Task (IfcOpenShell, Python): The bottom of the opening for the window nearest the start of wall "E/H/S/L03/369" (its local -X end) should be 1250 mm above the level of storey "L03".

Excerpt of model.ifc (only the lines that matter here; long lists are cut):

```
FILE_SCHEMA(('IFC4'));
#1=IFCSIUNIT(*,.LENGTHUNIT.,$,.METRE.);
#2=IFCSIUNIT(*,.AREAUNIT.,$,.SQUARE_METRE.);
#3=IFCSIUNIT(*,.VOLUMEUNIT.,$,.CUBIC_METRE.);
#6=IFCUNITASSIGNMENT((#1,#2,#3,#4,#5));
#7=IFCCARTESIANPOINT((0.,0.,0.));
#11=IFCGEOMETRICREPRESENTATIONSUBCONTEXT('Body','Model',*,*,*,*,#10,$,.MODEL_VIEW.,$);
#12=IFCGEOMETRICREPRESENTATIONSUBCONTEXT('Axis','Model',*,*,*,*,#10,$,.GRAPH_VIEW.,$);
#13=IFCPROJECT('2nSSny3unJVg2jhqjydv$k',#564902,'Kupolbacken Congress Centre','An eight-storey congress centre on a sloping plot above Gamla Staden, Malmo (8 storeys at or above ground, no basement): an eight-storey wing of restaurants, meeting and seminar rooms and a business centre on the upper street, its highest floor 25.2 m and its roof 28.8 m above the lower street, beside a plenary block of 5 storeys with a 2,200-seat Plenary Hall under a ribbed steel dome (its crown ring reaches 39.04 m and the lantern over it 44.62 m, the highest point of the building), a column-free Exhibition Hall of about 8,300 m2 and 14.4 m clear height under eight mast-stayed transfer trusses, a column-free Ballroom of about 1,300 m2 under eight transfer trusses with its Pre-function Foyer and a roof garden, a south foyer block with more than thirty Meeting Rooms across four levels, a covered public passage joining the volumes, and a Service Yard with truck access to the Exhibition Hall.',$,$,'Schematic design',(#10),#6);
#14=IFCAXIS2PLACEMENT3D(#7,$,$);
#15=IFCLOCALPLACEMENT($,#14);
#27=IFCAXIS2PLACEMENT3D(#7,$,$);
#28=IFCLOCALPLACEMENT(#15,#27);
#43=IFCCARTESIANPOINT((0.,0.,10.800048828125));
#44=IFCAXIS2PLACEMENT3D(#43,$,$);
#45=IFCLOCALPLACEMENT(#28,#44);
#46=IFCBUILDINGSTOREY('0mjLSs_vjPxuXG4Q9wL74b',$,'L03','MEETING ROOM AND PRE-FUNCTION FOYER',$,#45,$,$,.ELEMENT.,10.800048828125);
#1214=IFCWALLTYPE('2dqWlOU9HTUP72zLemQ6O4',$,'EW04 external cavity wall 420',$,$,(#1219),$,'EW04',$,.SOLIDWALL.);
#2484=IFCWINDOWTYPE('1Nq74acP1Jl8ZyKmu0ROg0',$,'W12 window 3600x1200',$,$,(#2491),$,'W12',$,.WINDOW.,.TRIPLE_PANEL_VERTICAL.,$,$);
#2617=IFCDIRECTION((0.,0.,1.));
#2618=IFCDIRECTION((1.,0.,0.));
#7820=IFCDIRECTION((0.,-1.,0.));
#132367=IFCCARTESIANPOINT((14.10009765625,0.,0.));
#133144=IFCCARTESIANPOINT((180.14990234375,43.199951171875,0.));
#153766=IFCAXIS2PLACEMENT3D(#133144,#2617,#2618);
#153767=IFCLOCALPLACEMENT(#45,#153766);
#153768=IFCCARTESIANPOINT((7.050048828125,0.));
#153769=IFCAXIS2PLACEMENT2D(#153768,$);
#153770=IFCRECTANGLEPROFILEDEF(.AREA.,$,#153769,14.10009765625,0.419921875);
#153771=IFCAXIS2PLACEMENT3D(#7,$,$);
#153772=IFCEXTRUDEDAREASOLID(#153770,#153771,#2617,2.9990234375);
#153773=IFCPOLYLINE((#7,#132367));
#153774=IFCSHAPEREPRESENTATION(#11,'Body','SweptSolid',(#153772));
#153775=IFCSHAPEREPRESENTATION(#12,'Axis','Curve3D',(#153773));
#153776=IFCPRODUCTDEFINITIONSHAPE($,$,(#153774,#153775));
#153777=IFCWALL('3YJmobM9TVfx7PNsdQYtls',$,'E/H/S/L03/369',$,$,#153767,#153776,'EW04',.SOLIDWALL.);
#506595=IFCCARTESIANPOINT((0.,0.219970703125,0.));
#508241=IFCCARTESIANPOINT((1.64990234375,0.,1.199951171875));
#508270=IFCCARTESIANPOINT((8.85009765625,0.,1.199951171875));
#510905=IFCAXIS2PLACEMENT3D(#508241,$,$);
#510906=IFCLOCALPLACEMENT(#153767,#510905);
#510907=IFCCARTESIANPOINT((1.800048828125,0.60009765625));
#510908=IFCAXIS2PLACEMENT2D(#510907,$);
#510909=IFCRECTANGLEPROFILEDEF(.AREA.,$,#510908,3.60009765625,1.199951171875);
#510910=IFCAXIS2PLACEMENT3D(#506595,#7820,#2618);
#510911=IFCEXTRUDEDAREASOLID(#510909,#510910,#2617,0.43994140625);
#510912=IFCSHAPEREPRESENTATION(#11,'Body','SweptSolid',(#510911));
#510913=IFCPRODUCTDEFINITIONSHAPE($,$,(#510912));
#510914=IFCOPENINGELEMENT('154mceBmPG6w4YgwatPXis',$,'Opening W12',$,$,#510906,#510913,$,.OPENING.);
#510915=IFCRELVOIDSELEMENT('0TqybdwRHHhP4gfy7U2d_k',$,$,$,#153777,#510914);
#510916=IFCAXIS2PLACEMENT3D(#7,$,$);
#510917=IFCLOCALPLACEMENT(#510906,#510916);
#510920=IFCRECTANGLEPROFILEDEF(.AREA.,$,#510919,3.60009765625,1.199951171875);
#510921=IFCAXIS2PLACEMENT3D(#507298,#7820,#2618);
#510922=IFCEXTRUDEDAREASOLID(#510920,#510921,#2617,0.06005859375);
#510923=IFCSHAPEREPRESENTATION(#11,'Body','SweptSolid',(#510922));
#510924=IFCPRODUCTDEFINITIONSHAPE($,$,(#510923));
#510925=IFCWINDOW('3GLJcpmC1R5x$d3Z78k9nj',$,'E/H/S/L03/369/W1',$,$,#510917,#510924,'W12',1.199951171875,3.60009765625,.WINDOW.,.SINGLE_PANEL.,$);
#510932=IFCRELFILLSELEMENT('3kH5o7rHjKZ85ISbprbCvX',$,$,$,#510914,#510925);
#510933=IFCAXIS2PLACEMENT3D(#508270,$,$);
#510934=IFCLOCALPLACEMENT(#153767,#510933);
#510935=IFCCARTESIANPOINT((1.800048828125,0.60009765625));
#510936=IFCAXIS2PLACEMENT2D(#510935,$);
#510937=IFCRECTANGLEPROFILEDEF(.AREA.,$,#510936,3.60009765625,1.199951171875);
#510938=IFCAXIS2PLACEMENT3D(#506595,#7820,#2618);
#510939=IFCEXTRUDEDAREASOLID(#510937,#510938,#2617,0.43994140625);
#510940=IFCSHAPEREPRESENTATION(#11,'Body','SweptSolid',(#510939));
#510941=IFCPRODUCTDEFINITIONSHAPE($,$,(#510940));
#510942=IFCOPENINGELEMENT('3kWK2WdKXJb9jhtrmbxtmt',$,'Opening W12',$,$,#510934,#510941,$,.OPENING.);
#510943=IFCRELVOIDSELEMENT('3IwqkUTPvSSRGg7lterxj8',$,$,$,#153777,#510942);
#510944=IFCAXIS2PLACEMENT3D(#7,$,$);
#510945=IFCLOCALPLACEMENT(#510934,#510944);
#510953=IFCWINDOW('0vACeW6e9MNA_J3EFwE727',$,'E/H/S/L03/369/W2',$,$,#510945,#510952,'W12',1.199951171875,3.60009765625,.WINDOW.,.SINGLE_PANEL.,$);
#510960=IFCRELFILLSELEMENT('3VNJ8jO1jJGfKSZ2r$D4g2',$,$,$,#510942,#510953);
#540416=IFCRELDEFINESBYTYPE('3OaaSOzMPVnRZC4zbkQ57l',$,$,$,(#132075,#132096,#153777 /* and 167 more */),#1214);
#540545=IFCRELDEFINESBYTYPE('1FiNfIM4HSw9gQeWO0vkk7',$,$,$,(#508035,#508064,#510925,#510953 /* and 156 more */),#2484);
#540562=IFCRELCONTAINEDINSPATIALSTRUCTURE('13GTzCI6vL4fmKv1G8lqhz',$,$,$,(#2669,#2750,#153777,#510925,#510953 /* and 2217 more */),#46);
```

```python
import numpy as np
import ifcopenshell
import ifcopenshell.api.geometry
import ifcopenshell.geom
import ifcopenshell.util.element
import ifcopenshell.util.placement
import ifcopenshell.util.shape
import ifcopenshell.util.unit

model = ifcopenshell.open("model.ifc")
unit_scale = ifcopenshell.util.unit.calculate_unit_scale(model)

window = model.by_id(510925)
opening = window.FillsVoids[0].RelatingOpeningElement
storey = ifcopenshell.util.element.get_container(window, ifc_class="IfcBuildingStorey")
level = ifcopenshell.util.placement.get_local_placement(storey.ObjectPlacement)[2, 3]

# The opening's origin need not be at the sill, so measure its lowest point.
shape = ifcopenshell.geom.create_shape(ifcopenshell.geom.settings(), opening)
bottom = ifcopenshell.util.shape.get_shape_bottom_elevation(shape, shape.geometry) / unit_scale
dz = level + 1.25 / unit_scale - bottom

shift = np.array([0.0, 0.0, dz])
# The window is placed relative to its opening, so it follows when the opening moves.
matrix = ifcopenshell.util.placement.get_local_placement(opening.ObjectPlacement)
matrix[:3, 3] += shift
ifcopenshell.api.geometry.edit_object_placement(
    model, product=opening, matrix=matrix, is_si=False, should_transform_children=True
)

print(f"moved by {dz * unit_scale:+.3f} m")

model.write("model_rev.ifc")
```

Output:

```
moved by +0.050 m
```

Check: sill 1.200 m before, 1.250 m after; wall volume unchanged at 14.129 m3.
